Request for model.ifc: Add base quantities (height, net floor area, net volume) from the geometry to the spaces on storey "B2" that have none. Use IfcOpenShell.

First a look at what the model holds.

```python
import ifcopenshell
import ifcopenshell.util.element
import ifcopenshell.util.unit

model = ifcopenshell.open("model.ifc")
print(model.schema)
for unit_type in ("LENGTHUNIT", "AREAUNIT", "VOLUMEUNIT"):
    print(unit_type, ifcopenshell.util.unit.calculate_unit_scale(model, unit_type))
storey = next(s for s in model.by_type("IfcBuildingStorey") if s.Name == "B2")
spaces = [e for e in ifcopenshell.util.element.get_decomposition(storey) if e.is_a("IfcSpace")]
for e in sorted(spaces, key=lambda e: e.id()):
    print(e.id(), e.is_a(), e.Name, list(ifcopenshell.util.element.get_psets(e, qtos_only=True)), sep=" | ")
```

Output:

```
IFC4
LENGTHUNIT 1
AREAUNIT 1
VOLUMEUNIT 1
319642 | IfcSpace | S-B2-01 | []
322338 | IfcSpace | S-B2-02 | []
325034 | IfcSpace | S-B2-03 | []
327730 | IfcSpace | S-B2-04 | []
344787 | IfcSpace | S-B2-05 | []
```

```python
import ifcopenshell
import ifcopenshell.api.pset
import ifcopenshell.geom
import ifcopenshell.util.element
import ifcopenshell.util.shape
import ifcopenshell.util.unit

model = ifcopenshell.open("model.ifc")
unit_scale = ifcopenshell.util.unit.calculate_unit_scale(model)
area_scale = ifcopenshell.util.unit.calculate_unit_scale(model, "AREAUNIT")
volume_scale = ifcopenshell.util.unit.calculate_unit_scale(model, "VOLUMEUNIT")
settings = ifcopenshell.geom.settings()

storey = next(s for s in model.by_type("IfcBuildingStorey") if s.Name == "B2")
spaces = [e for e in ifcopenshell.util.element.get_decomposition(storey) if e.is_a("IfcSpace")]

for e in sorted(spaces, key=lambda e: e.id()):
    if ifcopenshell.util.element.get_psets(e, qtos_only=True, should_inherit=False):
        continue
    # Geometry comes back in metres, in the element's own axes.
    shape = ifcopenshell.geom.create_shape(settings, e)
    values = {
        "Height": ifcopenshell.util.shape.get_z(shape.geometry) / unit_scale,
        "NetFloorArea": ifcopenshell.util.shape.get_footprint_area(shape.geometry) / area_scale,
        "NetVolume": ifcopenshell.util.shape.get_volume(shape.geometry) / volume_scale,
    }
    qto = ifcopenshell.api.pset.add_qto(model, product=e, name="Qto_SpaceBaseQuantities")
    ifcopenshell.api.pset.edit_qto(model, qto=qto, properties=values)
    print(e.id(), {k: round(v, 3) for k, v in values.items()})

model.write("model_updated.ifc")
```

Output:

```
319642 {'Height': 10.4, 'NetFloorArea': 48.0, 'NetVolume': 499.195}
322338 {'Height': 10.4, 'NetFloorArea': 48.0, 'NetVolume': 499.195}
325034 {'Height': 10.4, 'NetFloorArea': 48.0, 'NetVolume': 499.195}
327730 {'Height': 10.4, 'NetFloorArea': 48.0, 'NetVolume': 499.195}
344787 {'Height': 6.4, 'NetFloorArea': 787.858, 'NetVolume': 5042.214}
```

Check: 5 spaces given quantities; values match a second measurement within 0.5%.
